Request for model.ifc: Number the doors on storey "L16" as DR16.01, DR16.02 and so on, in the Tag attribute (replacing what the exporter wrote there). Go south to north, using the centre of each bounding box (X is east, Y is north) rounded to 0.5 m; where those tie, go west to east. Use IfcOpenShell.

First a look at what the model holds.

```python
import ifcopenshell
import ifcopenshell.util.element
import ifcopenshell.util.placement

model = ifcopenshell.open("model.ifc")
print(model.schema)
storey = next(s for s in model.by_type("IfcBuildingStorey") if s.Name == "L16")
doors = [e for e in ifcopenshell.util.element.get_decomposition(storey) if e.is_a("IfcDoor")]
for e in sorted(doors, key=lambda e: e.id()):
    origin = ifcopenshell.util.placement.get_local_placement(e.ObjectPlacement)[:3, 3]
    print(e.id(), e.Tag, e.Name, origin.round(2) + 0.0, sep=" | ")
```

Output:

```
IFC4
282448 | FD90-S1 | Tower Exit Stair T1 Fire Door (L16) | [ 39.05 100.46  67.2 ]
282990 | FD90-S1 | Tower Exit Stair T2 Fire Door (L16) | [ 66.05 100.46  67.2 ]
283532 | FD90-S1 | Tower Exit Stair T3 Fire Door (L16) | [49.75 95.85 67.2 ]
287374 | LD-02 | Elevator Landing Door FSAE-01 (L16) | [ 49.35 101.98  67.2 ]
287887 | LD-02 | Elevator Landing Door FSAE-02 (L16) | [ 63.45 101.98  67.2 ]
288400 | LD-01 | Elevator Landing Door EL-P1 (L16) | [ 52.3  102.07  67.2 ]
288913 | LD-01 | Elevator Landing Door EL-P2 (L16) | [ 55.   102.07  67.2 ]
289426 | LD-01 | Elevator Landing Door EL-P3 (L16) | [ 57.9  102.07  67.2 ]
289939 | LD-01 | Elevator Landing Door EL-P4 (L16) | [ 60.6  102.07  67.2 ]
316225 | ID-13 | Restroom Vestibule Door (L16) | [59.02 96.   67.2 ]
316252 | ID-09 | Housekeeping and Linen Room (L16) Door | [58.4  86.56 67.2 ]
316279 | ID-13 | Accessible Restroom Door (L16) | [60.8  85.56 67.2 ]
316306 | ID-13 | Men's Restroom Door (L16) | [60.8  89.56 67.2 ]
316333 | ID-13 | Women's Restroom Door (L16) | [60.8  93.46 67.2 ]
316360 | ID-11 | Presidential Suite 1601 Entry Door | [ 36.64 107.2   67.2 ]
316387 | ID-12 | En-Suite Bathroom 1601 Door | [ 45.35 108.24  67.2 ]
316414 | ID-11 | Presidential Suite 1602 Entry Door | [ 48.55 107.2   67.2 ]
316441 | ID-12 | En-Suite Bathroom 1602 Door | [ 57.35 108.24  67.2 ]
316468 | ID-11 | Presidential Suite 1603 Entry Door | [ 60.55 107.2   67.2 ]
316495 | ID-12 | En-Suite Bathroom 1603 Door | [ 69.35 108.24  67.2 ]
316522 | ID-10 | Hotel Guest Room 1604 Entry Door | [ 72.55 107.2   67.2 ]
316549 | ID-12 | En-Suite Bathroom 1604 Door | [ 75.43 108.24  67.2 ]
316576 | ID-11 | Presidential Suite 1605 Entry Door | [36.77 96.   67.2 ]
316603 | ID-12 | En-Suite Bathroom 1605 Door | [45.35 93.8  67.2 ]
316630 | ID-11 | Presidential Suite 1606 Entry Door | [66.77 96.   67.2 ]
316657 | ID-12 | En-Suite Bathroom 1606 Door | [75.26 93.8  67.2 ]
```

```python
import ifcopenshell
import ifcopenshell.geom
import ifcopenshell.util.element
import ifcopenshell.util.shape

model = ifcopenshell.open("model.ifc")
settings = ifcopenshell.geom.settings()
settings.set("use-world-coords", True)


def centre(element):
    shape = ifcopenshell.geom.create_shape(settings, element)
    return ifcopenshell.util.shape.get_bbox_centroid(shape.geometry)


storey = next(s for s in model.by_type("IfcBuildingStorey") if s.Name == "L16")
doors = [e for e in ifcopenshell.util.element.get_decomposition(storey) if e.is_a("IfcDoor")]

# Insertion points can sit at a corner or the storey origin, so sort by the geometry (in metres).
centres = {e: centre(e) for e in doors}
doors.sort(key=lambda e: (round(centres[e][1] / 0.5), centres[e][0]))

for i, e in enumerate(doors, start=1):
    number = f"DR16.{i:02d}"
    e.Tag = number
    print(e.id(), number)

model.write("model_updated.ifc")
```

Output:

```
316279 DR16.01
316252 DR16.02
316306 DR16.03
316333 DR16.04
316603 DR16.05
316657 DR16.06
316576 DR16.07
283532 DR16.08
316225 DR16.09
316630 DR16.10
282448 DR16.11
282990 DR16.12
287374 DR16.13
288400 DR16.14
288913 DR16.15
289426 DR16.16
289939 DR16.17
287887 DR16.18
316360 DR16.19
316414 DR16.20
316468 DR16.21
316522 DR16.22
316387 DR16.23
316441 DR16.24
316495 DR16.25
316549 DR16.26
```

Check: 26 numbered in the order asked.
